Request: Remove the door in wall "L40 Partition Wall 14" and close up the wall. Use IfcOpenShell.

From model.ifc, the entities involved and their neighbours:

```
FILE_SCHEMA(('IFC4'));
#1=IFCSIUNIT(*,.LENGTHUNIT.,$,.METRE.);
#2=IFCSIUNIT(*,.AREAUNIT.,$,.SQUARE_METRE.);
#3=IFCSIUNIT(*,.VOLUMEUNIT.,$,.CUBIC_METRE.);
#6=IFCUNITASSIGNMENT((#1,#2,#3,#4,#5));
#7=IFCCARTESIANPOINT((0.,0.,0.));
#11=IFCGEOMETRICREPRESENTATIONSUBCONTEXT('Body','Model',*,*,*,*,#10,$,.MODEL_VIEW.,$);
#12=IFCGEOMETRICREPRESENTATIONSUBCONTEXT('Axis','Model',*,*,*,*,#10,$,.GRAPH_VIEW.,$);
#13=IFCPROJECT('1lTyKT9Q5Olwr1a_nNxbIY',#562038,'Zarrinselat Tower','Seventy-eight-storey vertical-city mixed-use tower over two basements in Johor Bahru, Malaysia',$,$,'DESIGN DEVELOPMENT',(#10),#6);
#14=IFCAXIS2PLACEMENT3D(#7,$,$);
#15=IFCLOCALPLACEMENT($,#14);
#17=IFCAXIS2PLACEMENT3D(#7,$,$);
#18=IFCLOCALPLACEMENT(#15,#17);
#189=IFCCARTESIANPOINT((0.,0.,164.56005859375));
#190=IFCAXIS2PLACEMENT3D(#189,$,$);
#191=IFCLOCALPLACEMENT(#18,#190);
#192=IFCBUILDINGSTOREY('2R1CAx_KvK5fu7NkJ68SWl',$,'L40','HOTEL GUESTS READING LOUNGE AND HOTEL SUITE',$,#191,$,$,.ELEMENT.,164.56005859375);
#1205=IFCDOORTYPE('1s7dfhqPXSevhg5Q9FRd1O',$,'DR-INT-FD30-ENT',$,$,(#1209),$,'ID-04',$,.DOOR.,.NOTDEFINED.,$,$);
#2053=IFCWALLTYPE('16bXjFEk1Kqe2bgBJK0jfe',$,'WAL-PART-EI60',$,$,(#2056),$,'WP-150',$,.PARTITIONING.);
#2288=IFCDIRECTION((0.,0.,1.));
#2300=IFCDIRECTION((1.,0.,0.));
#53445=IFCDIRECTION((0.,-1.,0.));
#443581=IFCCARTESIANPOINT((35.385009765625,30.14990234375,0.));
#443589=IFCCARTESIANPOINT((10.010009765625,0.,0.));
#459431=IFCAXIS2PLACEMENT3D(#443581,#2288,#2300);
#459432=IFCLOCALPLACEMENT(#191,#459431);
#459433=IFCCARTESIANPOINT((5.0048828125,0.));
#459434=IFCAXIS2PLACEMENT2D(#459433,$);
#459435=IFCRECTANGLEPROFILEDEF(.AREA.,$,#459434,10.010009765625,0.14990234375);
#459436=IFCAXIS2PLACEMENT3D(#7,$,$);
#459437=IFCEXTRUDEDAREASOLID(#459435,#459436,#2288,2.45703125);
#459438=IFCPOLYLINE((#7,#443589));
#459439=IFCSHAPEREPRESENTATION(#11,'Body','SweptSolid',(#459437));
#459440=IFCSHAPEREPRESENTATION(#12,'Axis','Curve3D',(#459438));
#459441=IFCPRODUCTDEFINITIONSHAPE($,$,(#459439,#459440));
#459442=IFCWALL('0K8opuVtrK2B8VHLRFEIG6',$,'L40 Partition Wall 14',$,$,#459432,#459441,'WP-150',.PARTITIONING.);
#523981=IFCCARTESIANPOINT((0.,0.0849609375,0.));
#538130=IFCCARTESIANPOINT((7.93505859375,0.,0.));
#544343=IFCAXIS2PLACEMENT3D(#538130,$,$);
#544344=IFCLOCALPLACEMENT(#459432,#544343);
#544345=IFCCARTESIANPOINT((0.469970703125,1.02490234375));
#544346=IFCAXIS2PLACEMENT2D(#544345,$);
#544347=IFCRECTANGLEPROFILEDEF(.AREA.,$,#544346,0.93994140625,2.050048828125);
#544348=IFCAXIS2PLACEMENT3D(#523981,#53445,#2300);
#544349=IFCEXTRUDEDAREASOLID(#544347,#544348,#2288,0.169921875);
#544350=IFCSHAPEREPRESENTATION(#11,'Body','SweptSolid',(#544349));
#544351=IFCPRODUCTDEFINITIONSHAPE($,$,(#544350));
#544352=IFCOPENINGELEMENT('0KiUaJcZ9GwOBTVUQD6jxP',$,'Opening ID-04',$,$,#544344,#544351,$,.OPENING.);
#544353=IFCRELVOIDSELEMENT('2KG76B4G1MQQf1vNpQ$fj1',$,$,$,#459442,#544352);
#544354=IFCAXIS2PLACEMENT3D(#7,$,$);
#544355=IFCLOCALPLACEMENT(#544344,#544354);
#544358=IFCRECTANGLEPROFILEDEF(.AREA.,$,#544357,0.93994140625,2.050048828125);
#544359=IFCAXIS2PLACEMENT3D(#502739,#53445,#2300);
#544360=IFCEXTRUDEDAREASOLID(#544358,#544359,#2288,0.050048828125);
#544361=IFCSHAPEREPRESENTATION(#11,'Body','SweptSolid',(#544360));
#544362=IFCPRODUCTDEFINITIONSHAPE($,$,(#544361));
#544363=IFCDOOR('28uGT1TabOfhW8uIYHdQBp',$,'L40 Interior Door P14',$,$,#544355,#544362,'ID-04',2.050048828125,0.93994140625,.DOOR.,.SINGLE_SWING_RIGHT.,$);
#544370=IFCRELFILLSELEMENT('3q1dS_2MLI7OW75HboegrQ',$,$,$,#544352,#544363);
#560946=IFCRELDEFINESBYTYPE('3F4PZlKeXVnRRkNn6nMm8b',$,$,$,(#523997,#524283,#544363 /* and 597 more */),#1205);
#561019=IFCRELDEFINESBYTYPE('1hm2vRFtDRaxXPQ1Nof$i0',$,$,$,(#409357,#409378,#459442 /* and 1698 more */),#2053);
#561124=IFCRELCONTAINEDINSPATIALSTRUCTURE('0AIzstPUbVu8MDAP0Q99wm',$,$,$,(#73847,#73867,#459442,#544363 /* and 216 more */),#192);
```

```python
import ifcopenshell
import ifcopenshell.api.feature
import ifcopenshell.api.root
import ifcopenshell.geom
import ifcopenshell.util.shape

model = ifcopenshell.open("model.ifc")
settings = ifcopenshell.geom.settings()


def volume(element):
    """Net volume in cubic metres, openings subtracted."""
    shape = ifcopenshell.geom.create_shape(settings, element)
    return ifcopenshell.util.shape.get_volume(shape.geometry)


door = model.by_id(544363)
opening = door.FillsVoids[0].RelatingOpeningElement
wall = opening.VoidsElements[0].RelatingBuildingElement
before = volume(wall)

ifcopenshell.api.root.remove_product(model, product=door)
ifcopenshell.api.feature.remove_feature(model, feature=opening)

after = volume(wall)

print(f"wall volume {before:.3f} -> {after:.3f} m3")

model.write("model-out.ifc")
```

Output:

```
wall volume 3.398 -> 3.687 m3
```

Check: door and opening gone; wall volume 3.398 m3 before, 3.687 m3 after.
